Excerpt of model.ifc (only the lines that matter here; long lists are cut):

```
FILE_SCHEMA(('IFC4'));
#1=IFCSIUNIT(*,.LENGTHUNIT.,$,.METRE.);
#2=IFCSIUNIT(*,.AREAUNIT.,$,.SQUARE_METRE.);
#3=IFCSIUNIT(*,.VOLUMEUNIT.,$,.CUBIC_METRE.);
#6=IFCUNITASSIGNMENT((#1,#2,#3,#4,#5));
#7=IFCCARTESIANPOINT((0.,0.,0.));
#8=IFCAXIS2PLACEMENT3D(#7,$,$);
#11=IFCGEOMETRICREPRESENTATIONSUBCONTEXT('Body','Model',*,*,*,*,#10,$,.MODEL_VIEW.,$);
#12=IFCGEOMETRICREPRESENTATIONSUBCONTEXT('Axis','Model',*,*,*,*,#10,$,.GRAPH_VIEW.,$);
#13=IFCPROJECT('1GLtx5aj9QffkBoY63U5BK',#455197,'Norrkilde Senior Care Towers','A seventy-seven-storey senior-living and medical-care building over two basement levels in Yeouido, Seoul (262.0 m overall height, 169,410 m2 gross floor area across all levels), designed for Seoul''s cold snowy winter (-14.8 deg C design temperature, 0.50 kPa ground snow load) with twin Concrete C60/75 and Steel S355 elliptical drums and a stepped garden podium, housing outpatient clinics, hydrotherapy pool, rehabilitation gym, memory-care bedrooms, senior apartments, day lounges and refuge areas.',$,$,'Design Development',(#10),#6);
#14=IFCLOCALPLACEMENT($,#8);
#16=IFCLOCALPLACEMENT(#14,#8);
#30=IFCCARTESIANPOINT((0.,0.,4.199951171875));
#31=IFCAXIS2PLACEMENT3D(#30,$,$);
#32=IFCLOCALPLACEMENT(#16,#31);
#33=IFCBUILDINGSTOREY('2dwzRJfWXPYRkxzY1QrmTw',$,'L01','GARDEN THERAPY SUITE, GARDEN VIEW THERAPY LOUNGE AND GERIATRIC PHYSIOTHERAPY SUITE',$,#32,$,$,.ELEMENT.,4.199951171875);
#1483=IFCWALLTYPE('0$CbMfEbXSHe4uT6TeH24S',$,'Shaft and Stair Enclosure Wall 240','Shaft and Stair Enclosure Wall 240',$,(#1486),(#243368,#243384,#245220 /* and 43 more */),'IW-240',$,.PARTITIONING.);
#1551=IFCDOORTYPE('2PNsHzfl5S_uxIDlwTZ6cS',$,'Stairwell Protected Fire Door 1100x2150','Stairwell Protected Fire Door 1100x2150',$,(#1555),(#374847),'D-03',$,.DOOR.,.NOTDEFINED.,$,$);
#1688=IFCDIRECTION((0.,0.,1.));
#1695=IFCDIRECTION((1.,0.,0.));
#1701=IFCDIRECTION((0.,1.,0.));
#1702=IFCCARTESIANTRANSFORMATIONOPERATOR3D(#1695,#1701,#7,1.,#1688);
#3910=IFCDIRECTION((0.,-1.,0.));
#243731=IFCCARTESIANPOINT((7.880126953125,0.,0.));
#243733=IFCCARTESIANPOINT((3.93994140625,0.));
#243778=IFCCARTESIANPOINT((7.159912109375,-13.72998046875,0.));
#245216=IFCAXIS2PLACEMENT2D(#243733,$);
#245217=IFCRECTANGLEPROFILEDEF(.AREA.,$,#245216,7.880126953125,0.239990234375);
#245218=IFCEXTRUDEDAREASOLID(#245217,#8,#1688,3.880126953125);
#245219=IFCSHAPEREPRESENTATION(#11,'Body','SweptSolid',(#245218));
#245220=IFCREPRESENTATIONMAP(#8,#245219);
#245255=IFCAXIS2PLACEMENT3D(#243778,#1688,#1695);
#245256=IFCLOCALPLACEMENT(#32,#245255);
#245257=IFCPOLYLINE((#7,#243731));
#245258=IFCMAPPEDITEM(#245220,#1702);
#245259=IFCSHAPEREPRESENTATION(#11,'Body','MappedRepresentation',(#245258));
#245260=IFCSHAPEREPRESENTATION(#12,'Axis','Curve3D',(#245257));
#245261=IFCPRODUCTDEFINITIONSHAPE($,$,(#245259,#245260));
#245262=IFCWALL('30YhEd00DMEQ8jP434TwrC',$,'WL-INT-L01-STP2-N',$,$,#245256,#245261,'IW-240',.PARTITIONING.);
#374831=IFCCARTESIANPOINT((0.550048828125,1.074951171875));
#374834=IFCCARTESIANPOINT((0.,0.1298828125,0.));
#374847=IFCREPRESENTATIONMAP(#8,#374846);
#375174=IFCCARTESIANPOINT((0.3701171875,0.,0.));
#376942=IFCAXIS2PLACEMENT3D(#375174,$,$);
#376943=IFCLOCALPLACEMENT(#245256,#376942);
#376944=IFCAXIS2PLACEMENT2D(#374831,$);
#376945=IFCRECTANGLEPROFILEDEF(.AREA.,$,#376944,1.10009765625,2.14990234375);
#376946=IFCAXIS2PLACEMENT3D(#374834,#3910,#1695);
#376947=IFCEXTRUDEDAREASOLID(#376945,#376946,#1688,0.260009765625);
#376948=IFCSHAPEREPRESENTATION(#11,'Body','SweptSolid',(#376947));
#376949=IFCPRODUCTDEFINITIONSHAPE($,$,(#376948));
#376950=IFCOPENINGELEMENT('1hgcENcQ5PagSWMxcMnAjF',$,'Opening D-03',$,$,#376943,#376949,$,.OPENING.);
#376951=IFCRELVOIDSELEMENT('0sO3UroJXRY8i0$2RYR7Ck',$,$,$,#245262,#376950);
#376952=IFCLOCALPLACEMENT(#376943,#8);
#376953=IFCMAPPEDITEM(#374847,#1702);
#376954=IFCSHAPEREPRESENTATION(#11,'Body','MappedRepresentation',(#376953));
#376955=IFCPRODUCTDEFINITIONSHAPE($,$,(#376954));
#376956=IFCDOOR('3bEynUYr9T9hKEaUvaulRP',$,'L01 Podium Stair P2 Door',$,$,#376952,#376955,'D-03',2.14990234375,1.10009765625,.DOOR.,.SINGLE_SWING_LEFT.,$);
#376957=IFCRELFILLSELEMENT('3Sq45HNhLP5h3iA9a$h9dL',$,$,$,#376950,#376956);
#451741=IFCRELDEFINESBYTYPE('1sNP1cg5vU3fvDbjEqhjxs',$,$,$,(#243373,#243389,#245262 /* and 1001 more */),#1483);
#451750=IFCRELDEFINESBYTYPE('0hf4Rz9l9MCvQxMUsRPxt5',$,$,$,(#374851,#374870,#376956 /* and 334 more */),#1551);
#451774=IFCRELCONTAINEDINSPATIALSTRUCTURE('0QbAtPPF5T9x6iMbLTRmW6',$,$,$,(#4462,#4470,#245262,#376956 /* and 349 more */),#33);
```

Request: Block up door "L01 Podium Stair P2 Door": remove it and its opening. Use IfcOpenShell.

```python
import ifcopenshell
import ifcopenshell.api.feature
import ifcopenshell.api.root
import ifcopenshell.geom
import ifcopenshell.util.shape

model = ifcopenshell.open("model.ifc")
settings = ifcopenshell.geom.settings()


def volume(element):
    """Net volume in cubic metres, openings subtracted."""
    shape = ifcopenshell.geom.create_shape(settings, element)
    return ifcopenshell.util.shape.get_volume(shape.geometry)


door = model.by_guid("3bEynUYr9T9hKEaUvaulRP")
opening = door.FillsVoids[0].RelatingOpeningElement
wall = opening.VoidsElements[0].RelatingBuildingElement
before = volume(wall)

ifcopenshell.api.root.remove_product(model, product=door)
ifcopenshell.api.feature.remove_feature(model, feature=opening)

after = volume(wall)

print(f"wall volume {before:.3f} -> {after:.3f} m3")

model.write("model_rev.ifc")
```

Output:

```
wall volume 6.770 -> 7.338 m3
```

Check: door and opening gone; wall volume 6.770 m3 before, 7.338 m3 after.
